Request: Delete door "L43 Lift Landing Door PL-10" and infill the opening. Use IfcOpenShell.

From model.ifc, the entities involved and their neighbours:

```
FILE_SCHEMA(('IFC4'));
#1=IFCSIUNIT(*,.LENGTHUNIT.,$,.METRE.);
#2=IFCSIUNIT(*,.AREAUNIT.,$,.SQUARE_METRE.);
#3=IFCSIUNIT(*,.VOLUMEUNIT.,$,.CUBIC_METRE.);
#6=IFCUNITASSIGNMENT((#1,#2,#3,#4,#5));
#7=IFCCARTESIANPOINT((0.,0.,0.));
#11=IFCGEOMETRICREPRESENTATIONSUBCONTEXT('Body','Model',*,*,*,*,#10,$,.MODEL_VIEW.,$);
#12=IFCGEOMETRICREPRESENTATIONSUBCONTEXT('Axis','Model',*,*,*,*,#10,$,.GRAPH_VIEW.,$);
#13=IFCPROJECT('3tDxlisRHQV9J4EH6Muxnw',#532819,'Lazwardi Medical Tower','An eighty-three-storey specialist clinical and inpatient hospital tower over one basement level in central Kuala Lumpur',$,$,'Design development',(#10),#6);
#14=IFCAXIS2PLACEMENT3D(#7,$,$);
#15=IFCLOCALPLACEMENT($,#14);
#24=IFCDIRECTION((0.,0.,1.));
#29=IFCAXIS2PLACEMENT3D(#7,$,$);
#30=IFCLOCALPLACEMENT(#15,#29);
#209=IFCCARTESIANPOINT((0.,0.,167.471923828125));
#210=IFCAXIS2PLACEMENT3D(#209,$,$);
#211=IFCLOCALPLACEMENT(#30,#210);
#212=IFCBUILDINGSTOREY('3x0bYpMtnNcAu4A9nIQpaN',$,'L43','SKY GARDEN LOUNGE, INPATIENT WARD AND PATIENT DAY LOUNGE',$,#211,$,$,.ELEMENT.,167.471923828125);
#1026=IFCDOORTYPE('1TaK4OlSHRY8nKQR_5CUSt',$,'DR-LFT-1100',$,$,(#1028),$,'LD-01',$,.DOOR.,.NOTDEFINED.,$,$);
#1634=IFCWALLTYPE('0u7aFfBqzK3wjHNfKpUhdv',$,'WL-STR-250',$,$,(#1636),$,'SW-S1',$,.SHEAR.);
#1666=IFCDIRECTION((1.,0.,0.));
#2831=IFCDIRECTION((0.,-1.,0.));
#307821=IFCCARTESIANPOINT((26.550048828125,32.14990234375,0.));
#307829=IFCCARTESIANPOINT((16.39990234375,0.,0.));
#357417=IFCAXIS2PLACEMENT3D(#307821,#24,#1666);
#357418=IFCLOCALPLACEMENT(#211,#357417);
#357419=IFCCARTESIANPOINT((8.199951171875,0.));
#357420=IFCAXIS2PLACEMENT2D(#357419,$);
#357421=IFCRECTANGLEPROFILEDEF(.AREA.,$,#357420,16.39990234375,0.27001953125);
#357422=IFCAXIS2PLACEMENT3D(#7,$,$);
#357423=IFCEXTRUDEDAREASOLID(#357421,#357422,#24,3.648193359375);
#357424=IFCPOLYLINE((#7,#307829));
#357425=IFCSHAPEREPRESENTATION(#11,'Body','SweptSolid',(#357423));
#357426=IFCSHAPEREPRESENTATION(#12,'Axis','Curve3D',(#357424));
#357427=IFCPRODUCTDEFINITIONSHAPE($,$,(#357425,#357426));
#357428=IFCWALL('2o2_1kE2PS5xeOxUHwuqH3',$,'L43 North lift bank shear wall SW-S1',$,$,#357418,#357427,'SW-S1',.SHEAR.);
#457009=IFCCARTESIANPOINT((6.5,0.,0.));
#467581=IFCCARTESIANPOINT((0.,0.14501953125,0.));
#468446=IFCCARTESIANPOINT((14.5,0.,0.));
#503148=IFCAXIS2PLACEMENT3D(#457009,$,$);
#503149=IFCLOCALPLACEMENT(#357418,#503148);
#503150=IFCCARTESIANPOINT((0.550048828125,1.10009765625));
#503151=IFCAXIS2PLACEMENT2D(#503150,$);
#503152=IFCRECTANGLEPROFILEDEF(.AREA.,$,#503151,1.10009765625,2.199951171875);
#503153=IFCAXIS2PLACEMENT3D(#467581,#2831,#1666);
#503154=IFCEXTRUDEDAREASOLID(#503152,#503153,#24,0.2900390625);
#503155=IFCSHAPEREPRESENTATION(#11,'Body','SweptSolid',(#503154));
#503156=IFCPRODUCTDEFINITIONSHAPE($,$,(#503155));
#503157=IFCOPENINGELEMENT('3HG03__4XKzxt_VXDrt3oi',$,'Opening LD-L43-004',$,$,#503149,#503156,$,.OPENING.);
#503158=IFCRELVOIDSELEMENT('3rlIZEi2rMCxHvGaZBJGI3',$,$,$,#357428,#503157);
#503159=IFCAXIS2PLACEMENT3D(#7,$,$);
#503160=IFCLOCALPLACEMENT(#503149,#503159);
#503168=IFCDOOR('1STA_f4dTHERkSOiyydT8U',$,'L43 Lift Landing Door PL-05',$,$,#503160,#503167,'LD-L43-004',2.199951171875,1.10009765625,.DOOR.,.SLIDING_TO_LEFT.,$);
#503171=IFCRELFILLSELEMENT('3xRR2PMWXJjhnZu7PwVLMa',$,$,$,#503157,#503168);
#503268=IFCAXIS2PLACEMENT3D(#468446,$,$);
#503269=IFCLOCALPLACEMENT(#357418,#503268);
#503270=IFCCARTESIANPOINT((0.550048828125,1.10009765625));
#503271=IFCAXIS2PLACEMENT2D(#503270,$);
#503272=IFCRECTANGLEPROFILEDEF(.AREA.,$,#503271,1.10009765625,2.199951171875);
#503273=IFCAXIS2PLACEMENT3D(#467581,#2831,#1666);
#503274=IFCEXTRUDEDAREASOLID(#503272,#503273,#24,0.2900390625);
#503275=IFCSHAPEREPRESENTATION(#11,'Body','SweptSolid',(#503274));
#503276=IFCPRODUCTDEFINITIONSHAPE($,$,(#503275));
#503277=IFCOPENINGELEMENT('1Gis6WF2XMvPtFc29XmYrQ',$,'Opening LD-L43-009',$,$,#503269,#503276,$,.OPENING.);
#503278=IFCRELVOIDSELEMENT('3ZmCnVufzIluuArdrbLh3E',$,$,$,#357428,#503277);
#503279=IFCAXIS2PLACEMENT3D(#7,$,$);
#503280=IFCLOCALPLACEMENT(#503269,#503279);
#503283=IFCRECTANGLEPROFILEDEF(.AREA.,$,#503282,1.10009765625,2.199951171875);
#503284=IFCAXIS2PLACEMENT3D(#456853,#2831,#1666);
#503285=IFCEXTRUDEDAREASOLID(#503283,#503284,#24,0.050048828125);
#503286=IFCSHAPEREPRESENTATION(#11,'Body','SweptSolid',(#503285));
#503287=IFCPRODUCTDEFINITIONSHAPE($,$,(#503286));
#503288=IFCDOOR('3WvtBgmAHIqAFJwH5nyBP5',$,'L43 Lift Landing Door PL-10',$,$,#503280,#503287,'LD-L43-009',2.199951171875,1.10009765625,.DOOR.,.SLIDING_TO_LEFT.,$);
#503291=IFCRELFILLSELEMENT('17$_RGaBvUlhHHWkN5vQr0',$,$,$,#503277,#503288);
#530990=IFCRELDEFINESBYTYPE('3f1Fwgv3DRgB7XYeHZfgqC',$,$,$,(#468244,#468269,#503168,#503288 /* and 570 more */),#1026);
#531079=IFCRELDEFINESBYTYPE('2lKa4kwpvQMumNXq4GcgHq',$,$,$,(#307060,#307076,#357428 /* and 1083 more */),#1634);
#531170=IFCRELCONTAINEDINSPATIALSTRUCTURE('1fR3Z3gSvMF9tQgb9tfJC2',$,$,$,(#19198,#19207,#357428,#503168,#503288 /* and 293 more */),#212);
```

```python
import ifcopenshell
import ifcopenshell.api.feature
import ifcopenshell.api.root
import ifcopenshell.geom
import ifcopenshell.util.shape

model = ifcopenshell.open("model.ifc")
settings = ifcopenshell.geom.settings()


def volume(element):
    """Net volume in cubic metres, openings subtracted."""
    shape = ifcopenshell.geom.create_shape(settings, element)
    return ifcopenshell.util.shape.get_volume(shape.geometry)


door = model.by_id(503288)
opening = door.FillsVoids[0].RelatingOpeningElement
wall = opening.VoidsElements[0].RelatingBuildingElement
before = volume(wall)

ifcopenshell.api.root.remove_product(model, product=door)
ifcopenshell.api.feature.remove_feature(model, feature=opening)

after = volume(wall)

print(f"wall volume {before:.3f} -> {after:.3f} m3")

model.write("model_updated.ifc")
```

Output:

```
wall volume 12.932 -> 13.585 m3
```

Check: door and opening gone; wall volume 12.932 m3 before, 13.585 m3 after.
